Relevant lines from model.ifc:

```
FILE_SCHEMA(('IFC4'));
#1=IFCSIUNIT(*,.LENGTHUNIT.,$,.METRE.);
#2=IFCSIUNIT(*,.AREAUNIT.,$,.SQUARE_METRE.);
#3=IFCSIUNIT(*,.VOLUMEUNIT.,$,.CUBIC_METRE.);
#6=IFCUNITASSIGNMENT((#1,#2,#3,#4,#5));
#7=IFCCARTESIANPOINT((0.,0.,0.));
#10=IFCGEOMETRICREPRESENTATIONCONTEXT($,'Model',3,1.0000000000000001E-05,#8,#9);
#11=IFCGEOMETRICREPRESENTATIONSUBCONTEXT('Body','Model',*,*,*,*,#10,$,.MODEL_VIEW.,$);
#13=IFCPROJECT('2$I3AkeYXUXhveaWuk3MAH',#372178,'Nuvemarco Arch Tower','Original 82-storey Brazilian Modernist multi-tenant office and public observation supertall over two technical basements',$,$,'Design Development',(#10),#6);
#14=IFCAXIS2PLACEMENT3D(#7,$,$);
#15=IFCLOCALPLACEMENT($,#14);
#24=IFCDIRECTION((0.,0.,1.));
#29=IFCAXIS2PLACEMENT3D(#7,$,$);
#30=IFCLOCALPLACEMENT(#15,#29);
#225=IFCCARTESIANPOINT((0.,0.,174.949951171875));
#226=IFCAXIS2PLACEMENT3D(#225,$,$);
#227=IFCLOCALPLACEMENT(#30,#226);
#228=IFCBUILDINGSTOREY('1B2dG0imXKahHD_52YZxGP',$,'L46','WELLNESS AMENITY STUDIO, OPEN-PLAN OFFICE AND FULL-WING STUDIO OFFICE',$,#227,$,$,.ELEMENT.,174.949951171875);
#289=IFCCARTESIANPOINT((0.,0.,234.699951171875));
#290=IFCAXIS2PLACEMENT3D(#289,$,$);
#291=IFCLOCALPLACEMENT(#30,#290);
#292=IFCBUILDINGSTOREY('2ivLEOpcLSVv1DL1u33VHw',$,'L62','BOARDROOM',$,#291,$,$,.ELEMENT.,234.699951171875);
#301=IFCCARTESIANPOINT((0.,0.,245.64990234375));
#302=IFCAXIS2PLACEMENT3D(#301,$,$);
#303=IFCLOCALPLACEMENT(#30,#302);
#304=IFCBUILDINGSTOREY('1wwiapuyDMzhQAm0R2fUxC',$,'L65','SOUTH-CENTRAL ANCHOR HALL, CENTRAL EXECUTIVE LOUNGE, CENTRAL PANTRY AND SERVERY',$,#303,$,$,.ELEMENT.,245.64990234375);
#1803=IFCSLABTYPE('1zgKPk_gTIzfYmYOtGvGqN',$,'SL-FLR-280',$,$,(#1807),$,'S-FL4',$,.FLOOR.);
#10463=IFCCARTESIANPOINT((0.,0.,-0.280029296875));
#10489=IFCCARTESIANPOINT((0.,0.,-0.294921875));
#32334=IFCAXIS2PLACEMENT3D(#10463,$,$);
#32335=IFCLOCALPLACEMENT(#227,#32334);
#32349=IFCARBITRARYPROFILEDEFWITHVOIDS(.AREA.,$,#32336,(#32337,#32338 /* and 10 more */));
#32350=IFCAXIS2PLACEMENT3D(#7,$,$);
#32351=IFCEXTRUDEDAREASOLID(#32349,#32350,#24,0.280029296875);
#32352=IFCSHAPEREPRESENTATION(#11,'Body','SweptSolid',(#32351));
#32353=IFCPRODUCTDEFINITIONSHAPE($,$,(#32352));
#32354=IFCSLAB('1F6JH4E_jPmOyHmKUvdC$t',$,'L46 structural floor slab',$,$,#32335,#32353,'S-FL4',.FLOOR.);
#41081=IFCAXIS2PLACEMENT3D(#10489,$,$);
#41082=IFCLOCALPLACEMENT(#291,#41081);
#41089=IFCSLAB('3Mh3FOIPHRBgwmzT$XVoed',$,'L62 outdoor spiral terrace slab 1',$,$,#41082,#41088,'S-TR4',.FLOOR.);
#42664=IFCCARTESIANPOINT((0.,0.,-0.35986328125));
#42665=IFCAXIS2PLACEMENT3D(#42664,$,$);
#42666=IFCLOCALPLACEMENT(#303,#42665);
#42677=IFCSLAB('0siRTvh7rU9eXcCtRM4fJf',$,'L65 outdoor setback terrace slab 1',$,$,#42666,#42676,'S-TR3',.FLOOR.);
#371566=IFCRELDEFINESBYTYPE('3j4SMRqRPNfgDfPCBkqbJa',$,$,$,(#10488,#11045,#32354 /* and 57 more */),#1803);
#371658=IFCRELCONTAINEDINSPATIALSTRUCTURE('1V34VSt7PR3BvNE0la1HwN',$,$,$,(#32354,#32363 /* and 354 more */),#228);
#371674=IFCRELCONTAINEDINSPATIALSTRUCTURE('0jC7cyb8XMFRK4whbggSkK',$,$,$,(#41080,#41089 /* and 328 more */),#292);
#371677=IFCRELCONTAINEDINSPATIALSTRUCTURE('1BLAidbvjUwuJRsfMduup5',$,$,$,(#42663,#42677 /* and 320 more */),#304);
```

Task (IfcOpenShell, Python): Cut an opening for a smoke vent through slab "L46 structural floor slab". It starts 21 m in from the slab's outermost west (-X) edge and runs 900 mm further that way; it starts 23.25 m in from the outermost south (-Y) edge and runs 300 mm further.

```python
import numpy as np
import ifcopenshell
import ifcopenshell.api.feature
import ifcopenshell.api.geometry
import ifcopenshell.api.root
import ifcopenshell.geom
import ifcopenshell.util.placement
import ifcopenshell.util.representation
import ifcopenshell.util.shape
import ifcopenshell.util.unit

model = ifcopenshell.open("model.ifc")
unit_scale = ifcopenshell.util.unit.calculate_unit_scale(model)
settings = ifcopenshell.geom.settings()


def volume(element):
    """Net volume in cubic metres, openings subtracted."""
    shape = ifcopenshell.geom.create_shape(settings, element)
    return ifcopenshell.util.shape.get_volume(shape.geometry)


slab = model.by_guid("1F6JH4E_jPmOyHmKUvdC$t")
before = volume(slab)

# Extent in the slab's own axes, in metres. The edges named are its -X and -Y sides.
slab_shape = ifcopenshell.geom.create_shape(settings, slab)
vertices = ifcopenshell.util.shape.get_vertices(slab_shape.geometry)
x_min, y_min, bottom = vertices.min(axis=0)
top = vertices[:, 2].max()

opening = ifcopenshell.api.root.create_entity(model, ifc_class="IfcOpeningElement", name="Smoke vent opening", predefined_type="OPENING")
context = ifcopenshell.util.representation.get_context(model, "Model", "Body", "MODEL_VIEW")
width, depth = 0.9, 0.3
outline = [(0.0, 0.0), (width, 0.0), (width, depth), (0.0, depth), (0.0, 0.0)]
# Overshoot both faces by 50 mm so the cut is clean.
shape = ifcopenshell.api.geometry.add_slab_representation(
    model, context=context, depth=top - bottom + 0.1, polyline=outline
)
ifcopenshell.api.geometry.assign_representation(model, product=opening, representation=shape)

matrix = ifcopenshell.util.placement.get_local_placement(slab.ObjectPlacement)
matrix[:, 3] = matrix @ np.append(np.array([x_min + 21, y_min + 23.25, bottom - 0.05]) / unit_scale, 1.0)
ifcopenshell.api.geometry.edit_object_placement(model, product=opening, matrix=matrix, is_si=False)
ifcopenshell.api.feature.add_feature(model, feature=opening, element=slab)

after = volume(slab)

print(f"slab volume {before:.3f} -> {after:.3f} m3")

model.write("model_v2.ifc")
```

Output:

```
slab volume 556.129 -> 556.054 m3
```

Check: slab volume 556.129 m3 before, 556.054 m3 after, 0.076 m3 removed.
